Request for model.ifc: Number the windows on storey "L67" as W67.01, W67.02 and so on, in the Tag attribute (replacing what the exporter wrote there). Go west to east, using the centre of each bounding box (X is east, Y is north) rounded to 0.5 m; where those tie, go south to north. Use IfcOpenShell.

First a look at what the model holds.

```python
import ifcopenshell
import ifcopenshell.util.element
import ifcopenshell.util.placement

model = ifcopenshell.open("model.ifc")
print(model.schema)
storey = next(s for s in model.by_type("IfcBuildingStorey") if s.Name == "L67")
windows = [e for e in ifcopenshell.util.element.get_decomposition(storey) if e.is_a("IfcWindow")]
for e in sorted(windows, key=lambda e: e.id()):
    origin = ifcopenshell.util.placement.get_local_placement(e.ObjectPlacement)[:3, 3]
    print(e.id(), e.Tag, e.Name, origin.round(2) + 0.0, sep=" | ")
```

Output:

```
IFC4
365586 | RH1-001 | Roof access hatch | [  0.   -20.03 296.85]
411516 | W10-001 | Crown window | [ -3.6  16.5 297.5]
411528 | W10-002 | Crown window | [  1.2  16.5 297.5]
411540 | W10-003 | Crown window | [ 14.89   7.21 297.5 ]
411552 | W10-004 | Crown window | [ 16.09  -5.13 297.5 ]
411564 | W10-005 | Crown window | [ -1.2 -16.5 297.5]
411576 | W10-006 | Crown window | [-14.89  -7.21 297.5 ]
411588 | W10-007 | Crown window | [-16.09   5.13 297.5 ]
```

```python
import ifcopenshell
import ifcopenshell.geom
import ifcopenshell.util.element
import ifcopenshell.util.shape

model = ifcopenshell.open("model.ifc")
settings = ifcopenshell.geom.settings()
settings.set("use-world-coords", True)


def centre(element):
    shape = ifcopenshell.geom.create_shape(settings, element)
    return ifcopenshell.util.shape.get_bbox_centroid(shape.geometry)


storey = next(s for s in model.by_type("IfcBuildingStorey") if s.Name == "L67")
windows = [e for e in ifcopenshell.util.element.get_decomposition(storey) if e.is_a("IfcWindow")]

# Insertion points can sit at a corner or the storey origin, so sort by the geometry (in metres).
centres = {e: centre(e) for e in windows}
windows.sort(key=lambda e: (round(centres[e][0] / 0.5), centres[e][1]))

for i, e in enumerate(windows, start=1):
    number = f"W67.{i:02d}"
    e.Tag = number
    print(e.id(), number)

model.write("model_updated.ifc")
```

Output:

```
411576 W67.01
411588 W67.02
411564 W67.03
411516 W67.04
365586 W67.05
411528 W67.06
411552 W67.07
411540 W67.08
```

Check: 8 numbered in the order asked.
